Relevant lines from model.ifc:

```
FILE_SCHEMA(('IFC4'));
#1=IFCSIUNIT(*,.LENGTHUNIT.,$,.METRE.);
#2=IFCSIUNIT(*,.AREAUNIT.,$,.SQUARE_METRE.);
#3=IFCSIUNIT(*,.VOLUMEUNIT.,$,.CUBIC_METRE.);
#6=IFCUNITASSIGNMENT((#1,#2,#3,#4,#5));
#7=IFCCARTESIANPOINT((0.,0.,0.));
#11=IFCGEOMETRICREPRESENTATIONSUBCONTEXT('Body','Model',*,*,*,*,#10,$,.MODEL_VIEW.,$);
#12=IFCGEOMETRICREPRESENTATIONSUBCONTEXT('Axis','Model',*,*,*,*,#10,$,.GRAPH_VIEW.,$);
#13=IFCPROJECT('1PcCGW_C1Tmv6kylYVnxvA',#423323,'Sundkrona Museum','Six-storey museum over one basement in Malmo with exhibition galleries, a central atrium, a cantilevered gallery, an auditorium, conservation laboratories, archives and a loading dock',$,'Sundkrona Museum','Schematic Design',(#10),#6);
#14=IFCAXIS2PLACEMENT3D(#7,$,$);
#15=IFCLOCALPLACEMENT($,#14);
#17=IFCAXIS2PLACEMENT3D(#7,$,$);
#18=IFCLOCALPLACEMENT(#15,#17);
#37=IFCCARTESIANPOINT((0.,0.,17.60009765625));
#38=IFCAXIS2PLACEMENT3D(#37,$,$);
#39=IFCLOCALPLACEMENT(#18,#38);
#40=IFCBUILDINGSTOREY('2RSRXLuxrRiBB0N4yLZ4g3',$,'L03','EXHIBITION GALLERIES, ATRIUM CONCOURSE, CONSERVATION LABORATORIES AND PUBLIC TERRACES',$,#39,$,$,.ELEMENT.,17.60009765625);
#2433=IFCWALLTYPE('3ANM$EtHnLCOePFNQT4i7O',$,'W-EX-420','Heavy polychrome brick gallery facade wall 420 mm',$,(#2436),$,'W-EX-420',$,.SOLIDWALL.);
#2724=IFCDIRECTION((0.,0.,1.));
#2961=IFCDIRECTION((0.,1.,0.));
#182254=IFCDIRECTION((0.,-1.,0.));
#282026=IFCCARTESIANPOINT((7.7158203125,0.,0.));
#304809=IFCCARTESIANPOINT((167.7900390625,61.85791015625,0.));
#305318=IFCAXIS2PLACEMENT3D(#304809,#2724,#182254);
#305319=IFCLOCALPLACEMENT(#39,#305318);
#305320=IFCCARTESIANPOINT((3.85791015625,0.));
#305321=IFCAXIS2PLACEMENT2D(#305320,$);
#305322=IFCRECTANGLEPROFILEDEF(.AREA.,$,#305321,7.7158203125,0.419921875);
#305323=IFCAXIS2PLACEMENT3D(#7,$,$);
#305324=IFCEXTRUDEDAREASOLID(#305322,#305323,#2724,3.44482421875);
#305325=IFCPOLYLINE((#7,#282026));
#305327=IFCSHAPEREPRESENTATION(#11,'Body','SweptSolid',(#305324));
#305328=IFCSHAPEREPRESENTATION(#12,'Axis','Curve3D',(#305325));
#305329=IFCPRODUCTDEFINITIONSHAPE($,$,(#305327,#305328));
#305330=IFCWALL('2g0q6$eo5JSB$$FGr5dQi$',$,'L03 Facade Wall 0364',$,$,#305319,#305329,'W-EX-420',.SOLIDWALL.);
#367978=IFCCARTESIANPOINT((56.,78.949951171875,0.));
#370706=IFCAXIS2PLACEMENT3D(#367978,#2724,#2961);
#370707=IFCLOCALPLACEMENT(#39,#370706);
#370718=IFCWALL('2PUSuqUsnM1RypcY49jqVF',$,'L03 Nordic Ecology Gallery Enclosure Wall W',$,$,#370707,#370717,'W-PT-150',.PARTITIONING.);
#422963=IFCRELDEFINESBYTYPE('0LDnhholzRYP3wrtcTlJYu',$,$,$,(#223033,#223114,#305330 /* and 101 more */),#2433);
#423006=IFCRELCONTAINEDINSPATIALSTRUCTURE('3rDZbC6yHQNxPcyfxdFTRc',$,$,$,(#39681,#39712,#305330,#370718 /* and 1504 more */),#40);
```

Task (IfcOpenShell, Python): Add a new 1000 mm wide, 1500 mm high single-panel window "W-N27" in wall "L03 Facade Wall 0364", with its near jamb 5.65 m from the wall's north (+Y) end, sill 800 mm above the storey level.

```python
import numpy as np
import ifcopenshell
import ifcopenshell.api.feature
import ifcopenshell.api.geometry
import ifcopenshell.api.root
import ifcopenshell.api.spatial
import ifcopenshell.geom
import ifcopenshell.util.element
import ifcopenshell.util.placement
import ifcopenshell.util.representation
import ifcopenshell.util.shape
import ifcopenshell.util.unit

model = ifcopenshell.open("model.ifc")
unit_scale = ifcopenshell.util.unit.calculate_unit_scale(model)
settings = ifcopenshell.geom.settings()


def volume(element):
    """Net volume in cubic metres, openings subtracted."""
    shape = ifcopenshell.geom.create_shape(settings, element)
    return ifcopenshell.util.shape.get_volume(shape.geometry)


wall = model.by_guid("2g0q6$eo5JSB$$FGr5dQi$")
storey = ifcopenshell.util.element.get_container(wall, ifc_class="IfcBuildingStorey")
context = ifcopenshell.util.representation.get_context(model, "Model", "Body", "MODEL_VIEW")
before = volume(wall)

width, height, from_end, sill = 1, 1.5, 5.65, 0.8  # metres

# The wall runs along its own X axis, and the end named is its -X end.
wall_shape = ifcopenshell.geom.create_shape(settings, wall)
x, y, z = ifcopenshell.util.shape.get_vertices(wall_shape.geometry).T
start = x.min() + from_end
face, thickness = float(y.min()), float(y.max() - y.min())
wall_matrix = ifcopenshell.util.placement.get_local_placement(wall.ObjectPlacement)
level = ifcopenshell.util.placement.get_local_placement(storey.ObjectPlacement)[2, 3]


def in_wall(x, y):
    """Placement at x, y metres in the wall's axes, at sill height."""
    matrix = wall_matrix.copy()
    matrix[:, 3] = wall_matrix @ np.array([x / unit_scale, y / unit_scale, 0.0, 1.0])
    matrix[2, 3] = level + sill / unit_scale
    return matrix


# Opening: a box that overshoots both wall faces by 50 mm.
opening = ifcopenshell.api.root.create_entity(model, ifc_class="IfcOpeningElement", predefined_type="OPENING")
box = ifcopenshell.api.geometry.add_wall_representation(
    model, context=context, length=width, height=height, thickness=thickness + 0.1
)
ifcopenshell.api.geometry.assign_representation(model, product=opening, representation=box)
ifcopenshell.api.geometry.edit_object_placement(model, product=opening, matrix=in_wall(start, face - 0.05), is_si=False)
ifcopenshell.api.feature.add_feature(model, feature=opening, element=wall)

window = ifcopenshell.api.root.create_entity(model, ifc_class="IfcWindow", name="W-N27", predefined_type="WINDOW")
window.OverallWidth, window.OverallHeight = width / unit_scale, height / unit_scale
window.PartitioningType = "SINGLE_PANEL"
body = ifcopenshell.api.geometry.add_window_representation(
    model,
    context=context,
    overall_width=window.OverallWidth,
    overall_height=window.OverallHeight,
    partition_type="SINGLE_PANEL",
)
ifcopenshell.api.geometry.assign_representation(model, product=window, representation=body)
ifcopenshell.api.spatial.assign_container(model, products=[window], relating_structure=storey)
ifcopenshell.api.feature.add_filling(model, opening=opening, element=window)

# Centre the window in the wall's thickness.
ifcopenshell.api.geometry.edit_object_placement(model, product=window, matrix=in_wall(start, face), is_si=False)
window_shape = ifcopenshell.geom.create_shape(settings, window)
depth = ifcopenshell.util.shape.get_vertices(window_shape.geometry)[:, 1]
offset = face + thickness / 2 - (depth.min() + depth.max()) / 2
ifcopenshell.api.geometry.edit_object_placement(model, product=window, matrix=in_wall(start, offset), is_si=False)

after = volume(wall)

print(f"wall volume {before:.3f} -> {after:.3f} m3")

model.write("model-out.ifc")
```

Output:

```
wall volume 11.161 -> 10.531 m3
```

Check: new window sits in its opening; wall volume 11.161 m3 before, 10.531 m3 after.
